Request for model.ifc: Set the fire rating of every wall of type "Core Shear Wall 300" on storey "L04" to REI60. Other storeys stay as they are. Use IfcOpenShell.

First a look at what the model holds.

```python
import ifcopenshell
import ifcopenshell.util.element

model = ifcopenshell.open("model.ifc")
print(model.schema)
storey = next(s for s in model.by_type("IfcBuildingStorey") if s.Name == "L04")
walls = [e for e in ifcopenshell.util.element.get_decomposition(storey) if e.is_a("IfcWall")]
seen = {}
for e in walls:
    element_type = ifcopenshell.util.element.get_type(e)
    key = (element_type.Name if element_type != e and element_type else None, ifcopenshell.util.element.get_pset(e, "Pset_WallCommon", "FireRating"))
    seen[key] = seen.get(key, 0) + 1
for (name, value), count in sorted(seen.items(), key=str):
    print(count, "x", name, "|", value)
```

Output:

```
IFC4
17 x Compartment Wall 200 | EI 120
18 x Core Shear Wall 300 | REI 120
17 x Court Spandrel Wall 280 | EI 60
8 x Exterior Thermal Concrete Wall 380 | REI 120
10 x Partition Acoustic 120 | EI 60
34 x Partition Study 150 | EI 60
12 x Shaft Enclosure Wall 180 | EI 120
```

```python
import ifcopenshell
import ifcopenshell.api.pset
import ifcopenshell.util.element

model = ifcopenshell.open("model.ifc")

storey = next(s for s in model.by_type("IfcBuildingStorey") if s.Name == "L04")
walls = [e for e in ifcopenshell.util.element.get_decomposition(storey) if e.is_a("IfcWall")]

count = 0
for e in walls:
    element_type = ifcopenshell.util.element.get_type(e)
    if element_type in (None, e) or element_type.Name != "Core Shear Wall 300":
        continue
    # add_pset returns the element's existing set when there is one.
    pset = ifcopenshell.api.pset.add_pset(model, product=e, name="Pset_WallCommon")
    ifcopenshell.api.pset.edit_pset(model, pset=pset, properties={"FireRating": "REI60"})
    count += 1

print(count, "walls updated")

model.write("model-out.ifc")
```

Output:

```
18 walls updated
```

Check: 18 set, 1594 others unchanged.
